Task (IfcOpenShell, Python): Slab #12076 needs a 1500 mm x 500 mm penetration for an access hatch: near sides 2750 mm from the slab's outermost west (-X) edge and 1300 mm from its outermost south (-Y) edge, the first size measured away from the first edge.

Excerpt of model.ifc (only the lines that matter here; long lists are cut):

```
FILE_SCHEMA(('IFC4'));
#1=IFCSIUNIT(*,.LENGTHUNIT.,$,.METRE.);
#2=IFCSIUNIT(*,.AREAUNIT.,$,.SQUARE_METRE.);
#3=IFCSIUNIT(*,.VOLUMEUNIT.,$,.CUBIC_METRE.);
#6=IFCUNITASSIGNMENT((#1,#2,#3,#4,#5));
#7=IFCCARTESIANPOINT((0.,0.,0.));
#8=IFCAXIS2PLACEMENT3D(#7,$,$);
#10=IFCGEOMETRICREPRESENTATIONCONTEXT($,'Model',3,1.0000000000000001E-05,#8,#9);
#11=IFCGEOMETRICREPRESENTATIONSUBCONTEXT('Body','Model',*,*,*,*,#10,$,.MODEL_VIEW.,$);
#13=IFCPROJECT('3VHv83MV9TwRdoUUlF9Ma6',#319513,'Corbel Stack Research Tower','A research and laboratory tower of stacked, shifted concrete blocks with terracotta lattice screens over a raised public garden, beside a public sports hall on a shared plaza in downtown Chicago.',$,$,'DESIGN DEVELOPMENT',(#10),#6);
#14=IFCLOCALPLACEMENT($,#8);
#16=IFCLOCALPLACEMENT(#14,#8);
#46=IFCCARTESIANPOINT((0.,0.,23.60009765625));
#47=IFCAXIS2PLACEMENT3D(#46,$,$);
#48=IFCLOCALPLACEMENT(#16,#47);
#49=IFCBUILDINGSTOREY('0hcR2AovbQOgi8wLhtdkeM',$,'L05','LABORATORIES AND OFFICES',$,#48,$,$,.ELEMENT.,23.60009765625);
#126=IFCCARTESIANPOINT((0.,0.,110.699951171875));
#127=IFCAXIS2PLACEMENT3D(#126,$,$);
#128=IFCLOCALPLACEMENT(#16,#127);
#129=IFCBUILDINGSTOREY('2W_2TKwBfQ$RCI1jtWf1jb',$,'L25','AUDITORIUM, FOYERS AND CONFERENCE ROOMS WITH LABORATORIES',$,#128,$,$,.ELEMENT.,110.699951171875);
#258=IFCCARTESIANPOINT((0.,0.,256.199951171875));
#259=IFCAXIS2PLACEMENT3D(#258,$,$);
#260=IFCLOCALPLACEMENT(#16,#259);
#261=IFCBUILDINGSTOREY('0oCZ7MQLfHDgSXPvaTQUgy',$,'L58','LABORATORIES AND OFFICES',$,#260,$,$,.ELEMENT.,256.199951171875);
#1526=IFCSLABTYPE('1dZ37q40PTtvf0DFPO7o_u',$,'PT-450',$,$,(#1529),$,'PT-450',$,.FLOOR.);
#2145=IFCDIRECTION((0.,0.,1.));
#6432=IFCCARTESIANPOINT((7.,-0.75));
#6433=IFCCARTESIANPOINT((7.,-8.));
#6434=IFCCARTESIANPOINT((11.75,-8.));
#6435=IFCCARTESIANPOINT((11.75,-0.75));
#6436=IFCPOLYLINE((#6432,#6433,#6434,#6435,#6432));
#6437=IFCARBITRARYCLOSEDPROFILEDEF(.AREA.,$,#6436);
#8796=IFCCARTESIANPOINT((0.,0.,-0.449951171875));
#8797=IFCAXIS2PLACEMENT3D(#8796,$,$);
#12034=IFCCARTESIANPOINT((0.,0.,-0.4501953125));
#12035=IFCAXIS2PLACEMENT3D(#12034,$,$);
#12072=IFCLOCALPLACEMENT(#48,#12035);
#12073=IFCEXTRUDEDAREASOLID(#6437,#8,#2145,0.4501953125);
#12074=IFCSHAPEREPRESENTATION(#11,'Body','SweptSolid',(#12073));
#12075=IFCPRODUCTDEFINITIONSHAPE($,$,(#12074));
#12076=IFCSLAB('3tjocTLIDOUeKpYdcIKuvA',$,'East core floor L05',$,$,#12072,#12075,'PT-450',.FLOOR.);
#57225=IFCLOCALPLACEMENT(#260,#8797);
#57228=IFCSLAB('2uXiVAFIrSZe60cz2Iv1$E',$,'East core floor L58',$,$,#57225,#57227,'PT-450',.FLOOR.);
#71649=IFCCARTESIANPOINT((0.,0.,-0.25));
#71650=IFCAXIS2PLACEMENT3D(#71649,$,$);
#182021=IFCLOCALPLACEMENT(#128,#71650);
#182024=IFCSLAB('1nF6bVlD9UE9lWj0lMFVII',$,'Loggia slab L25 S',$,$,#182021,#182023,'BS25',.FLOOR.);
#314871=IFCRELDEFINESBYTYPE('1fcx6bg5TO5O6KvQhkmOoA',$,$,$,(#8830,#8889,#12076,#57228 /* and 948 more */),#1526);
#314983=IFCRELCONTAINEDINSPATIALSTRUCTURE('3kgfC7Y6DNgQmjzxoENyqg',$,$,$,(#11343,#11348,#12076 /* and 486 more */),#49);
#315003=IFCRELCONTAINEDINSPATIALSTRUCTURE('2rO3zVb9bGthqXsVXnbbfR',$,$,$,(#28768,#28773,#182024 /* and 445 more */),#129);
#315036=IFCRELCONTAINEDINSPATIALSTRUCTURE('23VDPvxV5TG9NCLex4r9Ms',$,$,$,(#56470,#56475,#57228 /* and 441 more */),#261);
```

```python
import numpy as np
import ifcopenshell
import ifcopenshell.api.feature
import ifcopenshell.api.geometry
import ifcopenshell.api.root
import ifcopenshell.geom
import ifcopenshell.util.placement
import ifcopenshell.util.representation
import ifcopenshell.util.shape
import ifcopenshell.util.unit

model = ifcopenshell.open("model.ifc")
unit_scale = ifcopenshell.util.unit.calculate_unit_scale(model)
settings = ifcopenshell.geom.settings()


def volume(element):
    """Net volume in cubic metres, openings subtracted."""
    shape = ifcopenshell.geom.create_shape(settings, element)
    return ifcopenshell.util.shape.get_volume(shape.geometry)


slab = model.by_guid("3tjocTLIDOUeKpYdcIKuvA")
before = volume(slab)

# Extent in the slab's own axes, in metres. The edges named are its -X and -Y sides.
slab_shape = ifcopenshell.geom.create_shape(settings, slab)
vertices = ifcopenshell.util.shape.get_vertices(slab_shape.geometry)
x_min, y_min, bottom = vertices.min(axis=0)
top = vertices[:, 2].max()

opening = ifcopenshell.api.root.create_entity(model, ifc_class="IfcOpeningElement", name="Access hatch opening", predefined_type="OPENING")
context = ifcopenshell.util.representation.get_context(model, "Model", "Body", "MODEL_VIEW")
width, depth = 1.5, 0.5
outline = [(0.0, 0.0), (width, 0.0), (width, depth), (0.0, depth), (0.0, 0.0)]
# Overshoot both faces by 50 mm so the cut is clean.
shape = ifcopenshell.api.geometry.add_slab_representation(
    model, context=context, depth=top - bottom + 0.1, polyline=outline
)
ifcopenshell.api.geometry.assign_representation(model, product=opening, representation=shape)

matrix = ifcopenshell.util.placement.get_local_placement(slab.ObjectPlacement)
matrix[:, 3] = matrix @ np.append(np.array([x_min + 2.75, y_min + 1.3, bottom - 0.05]) / unit_scale, 1.0)
ifcopenshell.api.geometry.edit_object_placement(model, product=opening, matrix=matrix, is_si=False)
ifcopenshell.api.feature.add_feature(model, feature=opening, element=slab)

after = volume(slab)

print(f"slab volume {before:.3f} -> {after:.3f} m3")

model.write("model_rev.ifc")
```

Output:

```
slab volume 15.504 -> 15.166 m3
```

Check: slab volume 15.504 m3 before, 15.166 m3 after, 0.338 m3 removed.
